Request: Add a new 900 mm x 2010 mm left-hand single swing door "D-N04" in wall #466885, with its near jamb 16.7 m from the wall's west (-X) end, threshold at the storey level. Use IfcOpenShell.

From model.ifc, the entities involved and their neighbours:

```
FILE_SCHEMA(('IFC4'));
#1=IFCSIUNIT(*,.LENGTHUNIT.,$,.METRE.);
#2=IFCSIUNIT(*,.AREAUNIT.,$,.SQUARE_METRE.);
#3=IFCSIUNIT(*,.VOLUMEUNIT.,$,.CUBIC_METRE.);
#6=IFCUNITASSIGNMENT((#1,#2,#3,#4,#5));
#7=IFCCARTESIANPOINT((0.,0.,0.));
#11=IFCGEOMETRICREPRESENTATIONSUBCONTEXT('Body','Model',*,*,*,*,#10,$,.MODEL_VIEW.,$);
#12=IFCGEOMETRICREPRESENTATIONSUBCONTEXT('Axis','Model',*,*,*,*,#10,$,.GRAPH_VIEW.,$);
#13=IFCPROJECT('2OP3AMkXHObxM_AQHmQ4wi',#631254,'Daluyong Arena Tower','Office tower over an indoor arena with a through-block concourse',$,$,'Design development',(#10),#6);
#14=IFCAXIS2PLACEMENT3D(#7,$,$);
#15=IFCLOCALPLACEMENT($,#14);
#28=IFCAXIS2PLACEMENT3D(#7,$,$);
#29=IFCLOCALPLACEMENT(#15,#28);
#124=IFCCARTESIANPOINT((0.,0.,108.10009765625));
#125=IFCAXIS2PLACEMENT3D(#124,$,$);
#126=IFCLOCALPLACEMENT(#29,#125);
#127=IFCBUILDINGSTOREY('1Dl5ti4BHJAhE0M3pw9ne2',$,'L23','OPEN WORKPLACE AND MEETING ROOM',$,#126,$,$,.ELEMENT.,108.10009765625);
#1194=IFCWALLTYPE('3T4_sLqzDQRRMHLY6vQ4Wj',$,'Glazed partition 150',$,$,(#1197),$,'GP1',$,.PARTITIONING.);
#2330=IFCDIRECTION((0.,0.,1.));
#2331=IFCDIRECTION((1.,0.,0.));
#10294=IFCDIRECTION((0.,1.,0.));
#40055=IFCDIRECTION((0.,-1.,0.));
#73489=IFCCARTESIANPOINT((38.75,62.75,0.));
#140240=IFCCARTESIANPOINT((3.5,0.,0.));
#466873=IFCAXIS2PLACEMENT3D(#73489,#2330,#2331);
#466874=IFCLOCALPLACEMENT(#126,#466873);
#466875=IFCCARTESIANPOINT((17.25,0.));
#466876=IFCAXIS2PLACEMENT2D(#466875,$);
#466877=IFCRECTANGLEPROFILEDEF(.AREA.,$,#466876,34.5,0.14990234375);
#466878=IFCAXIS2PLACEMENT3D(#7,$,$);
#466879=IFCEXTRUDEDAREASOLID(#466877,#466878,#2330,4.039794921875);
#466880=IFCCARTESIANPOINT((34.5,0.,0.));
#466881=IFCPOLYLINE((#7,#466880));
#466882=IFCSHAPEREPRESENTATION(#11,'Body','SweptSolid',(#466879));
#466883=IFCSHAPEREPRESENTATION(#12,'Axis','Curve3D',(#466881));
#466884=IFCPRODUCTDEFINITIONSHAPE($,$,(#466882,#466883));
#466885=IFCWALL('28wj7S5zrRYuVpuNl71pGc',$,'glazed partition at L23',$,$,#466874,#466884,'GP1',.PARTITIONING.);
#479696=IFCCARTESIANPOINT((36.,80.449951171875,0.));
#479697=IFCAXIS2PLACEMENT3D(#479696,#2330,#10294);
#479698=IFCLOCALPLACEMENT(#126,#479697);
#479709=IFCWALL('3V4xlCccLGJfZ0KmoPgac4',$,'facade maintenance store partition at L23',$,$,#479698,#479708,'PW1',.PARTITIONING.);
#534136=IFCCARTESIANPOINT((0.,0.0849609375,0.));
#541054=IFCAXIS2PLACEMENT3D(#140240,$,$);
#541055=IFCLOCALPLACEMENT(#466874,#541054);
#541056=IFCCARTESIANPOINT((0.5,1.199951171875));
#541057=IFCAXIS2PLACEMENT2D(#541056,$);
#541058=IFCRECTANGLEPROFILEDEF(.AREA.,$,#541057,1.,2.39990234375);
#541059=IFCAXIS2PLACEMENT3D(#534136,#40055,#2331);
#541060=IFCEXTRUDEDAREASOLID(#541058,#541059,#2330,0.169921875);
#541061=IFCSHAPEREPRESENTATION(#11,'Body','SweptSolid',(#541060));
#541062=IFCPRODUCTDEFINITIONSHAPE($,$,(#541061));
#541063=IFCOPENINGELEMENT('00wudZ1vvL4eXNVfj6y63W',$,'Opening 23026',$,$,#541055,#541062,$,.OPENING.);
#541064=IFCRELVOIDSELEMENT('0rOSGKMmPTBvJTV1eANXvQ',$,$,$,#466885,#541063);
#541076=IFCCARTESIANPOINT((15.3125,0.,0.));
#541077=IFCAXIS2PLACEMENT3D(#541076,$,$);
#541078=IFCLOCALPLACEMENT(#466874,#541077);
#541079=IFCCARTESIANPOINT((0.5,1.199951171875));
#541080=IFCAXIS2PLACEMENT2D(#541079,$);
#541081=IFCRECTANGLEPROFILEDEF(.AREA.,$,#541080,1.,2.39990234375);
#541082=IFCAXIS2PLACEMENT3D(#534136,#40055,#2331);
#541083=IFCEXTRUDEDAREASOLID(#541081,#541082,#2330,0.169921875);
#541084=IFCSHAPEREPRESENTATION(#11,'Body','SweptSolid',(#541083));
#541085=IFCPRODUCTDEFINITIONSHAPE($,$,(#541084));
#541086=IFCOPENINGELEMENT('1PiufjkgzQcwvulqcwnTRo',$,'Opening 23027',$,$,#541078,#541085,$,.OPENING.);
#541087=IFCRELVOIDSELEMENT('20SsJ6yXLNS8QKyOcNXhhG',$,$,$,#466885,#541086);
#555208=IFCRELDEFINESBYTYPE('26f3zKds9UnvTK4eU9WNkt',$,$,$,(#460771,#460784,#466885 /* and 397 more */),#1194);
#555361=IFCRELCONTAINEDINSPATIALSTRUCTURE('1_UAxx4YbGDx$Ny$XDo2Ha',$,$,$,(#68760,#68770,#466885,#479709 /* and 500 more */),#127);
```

```python
import numpy as np
import ifcopenshell
import ifcopenshell.api.feature
import ifcopenshell.api.geometry
import ifcopenshell.api.root
import ifcopenshell.api.spatial
import ifcopenshell.geom
import ifcopenshell.util.element
import ifcopenshell.util.placement
import ifcopenshell.util.representation
import ifcopenshell.util.shape
import ifcopenshell.util.unit

model = ifcopenshell.open("model.ifc")
unit_scale = ifcopenshell.util.unit.calculate_unit_scale(model)
settings = ifcopenshell.geom.settings()


def volume(element):
    """Net volume in cubic metres, openings subtracted."""
    shape = ifcopenshell.geom.create_shape(settings, element)
    return ifcopenshell.util.shape.get_volume(shape.geometry)


wall = model.by_guid("28wj7S5zrRYuVpuNl71pGc")
storey = ifcopenshell.util.element.get_container(wall, ifc_class="IfcBuildingStorey")
context = ifcopenshell.util.representation.get_context(model, "Model", "Body", "MODEL_VIEW")
before = volume(wall)

width, height, from_end, sill = 0.9, 2.01, 16.7, 0.0  # metres

# The wall runs along its own X axis, and the end named is its -X end.
wall_shape = ifcopenshell.geom.create_shape(settings, wall)
x, y, z = ifcopenshell.util.shape.get_vertices(wall_shape.geometry).T
start = x.min() + from_end
face, thickness = float(y.min()), float(y.max() - y.min())
wall_matrix = ifcopenshell.util.placement.get_local_placement(wall.ObjectPlacement)
level = ifcopenshell.util.placement.get_local_placement(storey.ObjectPlacement)[2, 3]


def in_wall(x, y):
    """Placement at x, y metres in the wall's axes, at sill height."""
    matrix = wall_matrix.copy()
    matrix[:, 3] = wall_matrix @ np.array([x / unit_scale, y / unit_scale, 0.0, 1.0])
    matrix[2, 3] = level + sill / unit_scale
    return matrix


# Opening: a box that overshoots both wall faces by 50 mm.
opening = ifcopenshell.api.root.create_entity(model, ifc_class="IfcOpeningElement", predefined_type="OPENING")
box = ifcopenshell.api.geometry.add_wall_representation(
    model, context=context, length=width, height=height, thickness=thickness + 0.1
)
ifcopenshell.api.geometry.assign_representation(model, product=opening, representation=box)
ifcopenshell.api.geometry.edit_object_placement(model, product=opening, matrix=in_wall(start, face - 0.05), is_si=False)
ifcopenshell.api.feature.add_feature(model, feature=opening, element=wall)

door = ifcopenshell.api.root.create_entity(model, ifc_class="IfcDoor", name="D-N04", predefined_type="DOOR")
door.OverallWidth, door.OverallHeight = width / unit_scale, height / unit_scale
door.OperationType = "SINGLE_SWING_LEFT"
body = ifcopenshell.api.geometry.add_door_representation(
    model,
    context=context,
    overall_width=door.OverallWidth,
    overall_height=door.OverallHeight,
    operation_type="SINGLE_SWING_LEFT",
    lining_properties={"LiningDepth": thickness / unit_scale, "ThresholdDepth": thickness / unit_scale},
)
ifcopenshell.api.geometry.assign_representation(model, product=door, representation=body)
ifcopenshell.api.spatial.assign_container(model, products=[door], relating_structure=storey)
ifcopenshell.api.feature.add_filling(model, opening=opening, element=door)

# The lining spans the wall, so the door starts at the wall face.
ifcopenshell.api.geometry.edit_object_placement(model, product=door, matrix=in_wall(start, face), is_si=False)

after = volume(wall)

print(f"wall volume {before:.3f} -> {after:.3f} m3")

model.write("model_updated.ifc")
```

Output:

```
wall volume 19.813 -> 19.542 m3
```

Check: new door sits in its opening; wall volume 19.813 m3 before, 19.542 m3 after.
